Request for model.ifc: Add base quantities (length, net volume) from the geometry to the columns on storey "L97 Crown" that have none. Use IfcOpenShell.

First a look at what the model holds.

```python
import ifcopenshell
import ifcopenshell.util.element
import ifcopenshell.util.unit

model = ifcopenshell.open("model.ifc")
print(model.schema)
for unit_type in ("LENGTHUNIT", "AREAUNIT", "VOLUMEUNIT"):
    print(unit_type, ifcopenshell.util.unit.calculate_unit_scale(model, unit_type))
storey = next(s for s in model.by_type("IfcBuildingStorey") if s.Name == "L97 Crown")
columns = [e for e in ifcopenshell.util.element.get_decomposition(storey) if e.is_a("IfcColumn")]
for e in sorted(columns, key=lambda e: e.id()):
    print(e.id(), e.is_a(), e.Name, list(ifcopenshell.util.element.get_psets(e, qtos_only=True)), sep=" | ")
```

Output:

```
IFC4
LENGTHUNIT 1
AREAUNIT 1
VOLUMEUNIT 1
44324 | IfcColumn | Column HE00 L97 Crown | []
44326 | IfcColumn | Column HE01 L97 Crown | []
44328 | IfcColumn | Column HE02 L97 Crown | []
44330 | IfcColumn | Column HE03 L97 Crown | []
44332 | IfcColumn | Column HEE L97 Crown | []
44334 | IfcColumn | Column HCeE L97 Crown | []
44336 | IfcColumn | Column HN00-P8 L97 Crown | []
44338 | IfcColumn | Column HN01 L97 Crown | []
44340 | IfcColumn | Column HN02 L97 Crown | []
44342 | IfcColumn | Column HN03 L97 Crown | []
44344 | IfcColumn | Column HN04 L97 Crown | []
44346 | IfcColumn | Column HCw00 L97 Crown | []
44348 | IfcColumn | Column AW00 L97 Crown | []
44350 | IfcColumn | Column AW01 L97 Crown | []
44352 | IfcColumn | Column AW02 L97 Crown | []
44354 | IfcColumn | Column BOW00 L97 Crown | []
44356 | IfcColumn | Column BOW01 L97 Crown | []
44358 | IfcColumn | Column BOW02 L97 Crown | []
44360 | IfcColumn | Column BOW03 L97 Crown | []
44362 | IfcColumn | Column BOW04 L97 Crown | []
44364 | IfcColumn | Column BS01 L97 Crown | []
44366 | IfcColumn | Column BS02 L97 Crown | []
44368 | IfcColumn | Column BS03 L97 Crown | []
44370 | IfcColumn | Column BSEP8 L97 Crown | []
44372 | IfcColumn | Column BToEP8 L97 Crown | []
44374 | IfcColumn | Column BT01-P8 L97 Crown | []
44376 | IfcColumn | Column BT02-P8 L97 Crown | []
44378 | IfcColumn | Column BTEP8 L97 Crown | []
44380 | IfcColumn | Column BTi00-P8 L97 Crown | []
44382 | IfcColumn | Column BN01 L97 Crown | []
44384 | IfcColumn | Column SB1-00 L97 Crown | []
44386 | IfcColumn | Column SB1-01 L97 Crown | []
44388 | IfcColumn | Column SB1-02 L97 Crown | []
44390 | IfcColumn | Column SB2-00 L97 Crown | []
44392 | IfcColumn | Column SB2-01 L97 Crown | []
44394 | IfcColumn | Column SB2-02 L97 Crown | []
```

```python
import ifcopenshell
import ifcopenshell.api.pset
import ifcopenshell.geom
import ifcopenshell.util.element
import ifcopenshell.util.shape
import ifcopenshell.util.unit

model = ifcopenshell.open("model.ifc")
unit_scale = ifcopenshell.util.unit.calculate_unit_scale(model)
volume_scale = ifcopenshell.util.unit.calculate_unit_scale(model, "VOLUMEUNIT")
settings = ifcopenshell.geom.settings()

storey = next(s for s in model.by_type("IfcBuildingStorey") if s.Name == "L97 Crown")
columns = [e for e in ifcopenshell.util.element.get_decomposition(storey) if e.is_a("IfcColumn")]

for e in sorted(columns, key=lambda e: e.id()):
    if ifcopenshell.util.element.get_psets(e, qtos_only=True, should_inherit=False):
        continue
    # Geometry comes back in metres, in the element's own axes.
    shape = ifcopenshell.geom.create_shape(settings, e)
    values = {
        "Length": ifcopenshell.util.shape.get_z(shape.geometry) / unit_scale,
        "NetVolume": ifcopenshell.util.shape.get_volume(shape.geometry) / volume_scale,
    }
    qto = ifcopenshell.api.pset.add_qto(model, product=e, name="Qto_ColumnBaseQuantities")
    ifcopenshell.api.pset.edit_qto(model, qto=qto, properties=values)
    print(e.id(), {k: round(v, 3) for k, v in values.items()})

model.write("model-out.ifc")
```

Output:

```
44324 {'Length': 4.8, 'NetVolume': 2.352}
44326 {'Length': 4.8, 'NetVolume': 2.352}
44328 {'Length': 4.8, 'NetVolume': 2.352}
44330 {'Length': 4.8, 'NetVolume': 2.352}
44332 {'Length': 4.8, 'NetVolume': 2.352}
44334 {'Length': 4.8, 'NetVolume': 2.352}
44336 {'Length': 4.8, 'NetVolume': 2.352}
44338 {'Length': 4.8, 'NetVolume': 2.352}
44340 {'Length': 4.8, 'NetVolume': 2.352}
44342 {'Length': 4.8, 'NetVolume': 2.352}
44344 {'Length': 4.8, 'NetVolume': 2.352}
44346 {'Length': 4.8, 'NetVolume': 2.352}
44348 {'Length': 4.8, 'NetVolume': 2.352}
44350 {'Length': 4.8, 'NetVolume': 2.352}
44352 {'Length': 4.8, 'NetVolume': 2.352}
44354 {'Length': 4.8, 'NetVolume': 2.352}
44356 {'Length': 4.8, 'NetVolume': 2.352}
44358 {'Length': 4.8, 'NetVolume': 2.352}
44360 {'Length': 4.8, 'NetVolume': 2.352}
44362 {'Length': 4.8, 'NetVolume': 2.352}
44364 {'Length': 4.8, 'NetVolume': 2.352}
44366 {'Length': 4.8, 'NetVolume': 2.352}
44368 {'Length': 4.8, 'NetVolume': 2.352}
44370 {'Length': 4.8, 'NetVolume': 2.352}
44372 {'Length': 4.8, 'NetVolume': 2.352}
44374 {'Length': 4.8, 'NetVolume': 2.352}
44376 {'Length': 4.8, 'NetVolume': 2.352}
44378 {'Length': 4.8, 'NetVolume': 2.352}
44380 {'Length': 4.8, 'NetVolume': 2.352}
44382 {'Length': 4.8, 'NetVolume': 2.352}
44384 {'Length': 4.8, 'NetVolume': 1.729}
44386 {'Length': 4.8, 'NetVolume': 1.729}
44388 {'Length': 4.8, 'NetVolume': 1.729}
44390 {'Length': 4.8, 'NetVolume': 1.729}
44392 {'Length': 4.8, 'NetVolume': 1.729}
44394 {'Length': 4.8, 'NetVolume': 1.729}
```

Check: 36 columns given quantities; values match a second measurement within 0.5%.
